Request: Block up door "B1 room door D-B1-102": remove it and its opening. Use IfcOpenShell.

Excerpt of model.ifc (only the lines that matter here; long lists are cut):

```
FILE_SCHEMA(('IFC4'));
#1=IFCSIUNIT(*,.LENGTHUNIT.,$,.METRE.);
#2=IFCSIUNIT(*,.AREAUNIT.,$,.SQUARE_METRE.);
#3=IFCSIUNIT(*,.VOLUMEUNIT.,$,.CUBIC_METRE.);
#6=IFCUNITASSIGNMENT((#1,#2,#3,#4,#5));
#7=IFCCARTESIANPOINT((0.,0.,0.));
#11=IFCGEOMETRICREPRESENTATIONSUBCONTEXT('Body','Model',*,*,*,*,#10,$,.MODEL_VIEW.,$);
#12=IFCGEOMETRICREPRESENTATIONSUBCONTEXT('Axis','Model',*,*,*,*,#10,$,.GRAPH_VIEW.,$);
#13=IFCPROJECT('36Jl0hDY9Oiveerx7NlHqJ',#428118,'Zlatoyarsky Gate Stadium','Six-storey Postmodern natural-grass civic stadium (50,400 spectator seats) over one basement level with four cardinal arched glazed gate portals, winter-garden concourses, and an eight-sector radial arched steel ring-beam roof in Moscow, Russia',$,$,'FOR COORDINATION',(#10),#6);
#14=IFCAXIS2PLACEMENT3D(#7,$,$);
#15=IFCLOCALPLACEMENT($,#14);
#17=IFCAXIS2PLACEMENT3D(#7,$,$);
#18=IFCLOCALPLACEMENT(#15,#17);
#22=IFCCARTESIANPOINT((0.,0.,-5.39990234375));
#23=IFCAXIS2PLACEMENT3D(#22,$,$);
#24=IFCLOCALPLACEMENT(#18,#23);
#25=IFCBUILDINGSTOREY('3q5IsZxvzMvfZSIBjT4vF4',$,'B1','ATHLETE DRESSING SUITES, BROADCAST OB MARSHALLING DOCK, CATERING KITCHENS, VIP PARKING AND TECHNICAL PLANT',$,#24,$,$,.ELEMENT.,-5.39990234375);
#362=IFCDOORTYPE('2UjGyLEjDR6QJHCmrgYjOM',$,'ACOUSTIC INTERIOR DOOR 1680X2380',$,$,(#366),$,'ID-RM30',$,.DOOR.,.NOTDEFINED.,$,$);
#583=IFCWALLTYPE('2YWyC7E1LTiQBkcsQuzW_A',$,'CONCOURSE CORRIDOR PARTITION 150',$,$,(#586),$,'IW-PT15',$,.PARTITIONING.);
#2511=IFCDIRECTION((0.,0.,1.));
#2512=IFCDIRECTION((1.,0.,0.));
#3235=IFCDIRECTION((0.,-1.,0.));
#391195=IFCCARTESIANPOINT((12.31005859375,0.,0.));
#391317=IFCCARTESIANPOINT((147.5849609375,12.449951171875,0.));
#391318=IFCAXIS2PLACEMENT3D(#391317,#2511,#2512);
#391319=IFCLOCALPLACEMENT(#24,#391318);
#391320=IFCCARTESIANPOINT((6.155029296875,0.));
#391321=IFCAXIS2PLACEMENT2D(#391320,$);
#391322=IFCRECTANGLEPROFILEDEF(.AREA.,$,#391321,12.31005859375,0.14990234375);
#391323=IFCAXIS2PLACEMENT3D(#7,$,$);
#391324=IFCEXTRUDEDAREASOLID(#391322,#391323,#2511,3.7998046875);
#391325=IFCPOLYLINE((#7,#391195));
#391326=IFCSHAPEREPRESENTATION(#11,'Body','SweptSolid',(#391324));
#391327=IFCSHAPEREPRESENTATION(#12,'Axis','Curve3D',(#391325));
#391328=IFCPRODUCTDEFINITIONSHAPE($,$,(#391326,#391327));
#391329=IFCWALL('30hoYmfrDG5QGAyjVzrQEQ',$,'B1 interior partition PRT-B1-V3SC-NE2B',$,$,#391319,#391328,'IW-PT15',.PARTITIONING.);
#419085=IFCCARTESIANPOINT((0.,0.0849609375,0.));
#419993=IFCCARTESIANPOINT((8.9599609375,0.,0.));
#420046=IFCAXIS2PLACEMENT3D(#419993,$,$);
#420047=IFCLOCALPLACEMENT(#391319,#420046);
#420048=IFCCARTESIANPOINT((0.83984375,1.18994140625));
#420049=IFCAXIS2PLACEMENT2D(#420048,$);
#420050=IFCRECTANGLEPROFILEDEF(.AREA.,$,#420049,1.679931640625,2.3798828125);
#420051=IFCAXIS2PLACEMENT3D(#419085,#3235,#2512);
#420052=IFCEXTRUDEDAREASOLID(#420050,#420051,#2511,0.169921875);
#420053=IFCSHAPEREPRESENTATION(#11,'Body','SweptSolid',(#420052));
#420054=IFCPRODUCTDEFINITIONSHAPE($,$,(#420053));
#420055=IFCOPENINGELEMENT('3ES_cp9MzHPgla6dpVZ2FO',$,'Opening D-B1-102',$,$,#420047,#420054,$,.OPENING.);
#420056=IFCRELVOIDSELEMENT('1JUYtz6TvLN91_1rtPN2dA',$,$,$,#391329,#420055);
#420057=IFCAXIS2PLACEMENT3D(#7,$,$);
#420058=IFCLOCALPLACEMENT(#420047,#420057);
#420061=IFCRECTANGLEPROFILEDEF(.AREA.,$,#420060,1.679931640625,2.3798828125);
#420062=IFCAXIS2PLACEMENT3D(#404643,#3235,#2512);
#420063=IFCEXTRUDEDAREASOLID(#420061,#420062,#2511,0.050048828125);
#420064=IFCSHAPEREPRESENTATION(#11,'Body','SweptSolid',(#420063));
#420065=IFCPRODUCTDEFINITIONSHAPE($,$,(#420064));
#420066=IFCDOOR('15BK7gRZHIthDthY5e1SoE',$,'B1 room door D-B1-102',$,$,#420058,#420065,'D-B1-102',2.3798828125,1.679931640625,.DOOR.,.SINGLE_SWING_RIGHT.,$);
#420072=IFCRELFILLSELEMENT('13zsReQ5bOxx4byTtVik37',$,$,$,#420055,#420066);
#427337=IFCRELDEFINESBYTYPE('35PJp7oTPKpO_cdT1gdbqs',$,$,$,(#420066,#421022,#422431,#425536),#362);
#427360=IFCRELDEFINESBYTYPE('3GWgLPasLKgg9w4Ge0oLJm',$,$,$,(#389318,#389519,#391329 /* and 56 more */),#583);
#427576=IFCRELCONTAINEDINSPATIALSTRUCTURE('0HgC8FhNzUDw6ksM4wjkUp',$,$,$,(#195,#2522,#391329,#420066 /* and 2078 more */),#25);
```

```python
import ifcopenshell
import ifcopenshell.api.feature
import ifcopenshell.api.root
import ifcopenshell.geom
import ifcopenshell.util.shape

model = ifcopenshell.open("model.ifc")
settings = ifcopenshell.geom.settings()


def volume(element):
    """Net volume in cubic metres, openings subtracted."""
    shape = ifcopenshell.geom.create_shape(settings, element)
    return ifcopenshell.util.shape.get_volume(shape.geometry)


door = model.by_id(420066)
opening = door.FillsVoids[0].RelatingOpeningElement
wall = opening.VoidsElements[0].RelatingBuildingElement
before = volume(wall)

ifcopenshell.api.root.remove_product(model, product=door)
ifcopenshell.api.feature.remove_feature(model, feature=opening)

after = volume(wall)

print(f"wall volume {before:.3f} -> {after:.3f} m3")

model.write("model_edited.ifc")
```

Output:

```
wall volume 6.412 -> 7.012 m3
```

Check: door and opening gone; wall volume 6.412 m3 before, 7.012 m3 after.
